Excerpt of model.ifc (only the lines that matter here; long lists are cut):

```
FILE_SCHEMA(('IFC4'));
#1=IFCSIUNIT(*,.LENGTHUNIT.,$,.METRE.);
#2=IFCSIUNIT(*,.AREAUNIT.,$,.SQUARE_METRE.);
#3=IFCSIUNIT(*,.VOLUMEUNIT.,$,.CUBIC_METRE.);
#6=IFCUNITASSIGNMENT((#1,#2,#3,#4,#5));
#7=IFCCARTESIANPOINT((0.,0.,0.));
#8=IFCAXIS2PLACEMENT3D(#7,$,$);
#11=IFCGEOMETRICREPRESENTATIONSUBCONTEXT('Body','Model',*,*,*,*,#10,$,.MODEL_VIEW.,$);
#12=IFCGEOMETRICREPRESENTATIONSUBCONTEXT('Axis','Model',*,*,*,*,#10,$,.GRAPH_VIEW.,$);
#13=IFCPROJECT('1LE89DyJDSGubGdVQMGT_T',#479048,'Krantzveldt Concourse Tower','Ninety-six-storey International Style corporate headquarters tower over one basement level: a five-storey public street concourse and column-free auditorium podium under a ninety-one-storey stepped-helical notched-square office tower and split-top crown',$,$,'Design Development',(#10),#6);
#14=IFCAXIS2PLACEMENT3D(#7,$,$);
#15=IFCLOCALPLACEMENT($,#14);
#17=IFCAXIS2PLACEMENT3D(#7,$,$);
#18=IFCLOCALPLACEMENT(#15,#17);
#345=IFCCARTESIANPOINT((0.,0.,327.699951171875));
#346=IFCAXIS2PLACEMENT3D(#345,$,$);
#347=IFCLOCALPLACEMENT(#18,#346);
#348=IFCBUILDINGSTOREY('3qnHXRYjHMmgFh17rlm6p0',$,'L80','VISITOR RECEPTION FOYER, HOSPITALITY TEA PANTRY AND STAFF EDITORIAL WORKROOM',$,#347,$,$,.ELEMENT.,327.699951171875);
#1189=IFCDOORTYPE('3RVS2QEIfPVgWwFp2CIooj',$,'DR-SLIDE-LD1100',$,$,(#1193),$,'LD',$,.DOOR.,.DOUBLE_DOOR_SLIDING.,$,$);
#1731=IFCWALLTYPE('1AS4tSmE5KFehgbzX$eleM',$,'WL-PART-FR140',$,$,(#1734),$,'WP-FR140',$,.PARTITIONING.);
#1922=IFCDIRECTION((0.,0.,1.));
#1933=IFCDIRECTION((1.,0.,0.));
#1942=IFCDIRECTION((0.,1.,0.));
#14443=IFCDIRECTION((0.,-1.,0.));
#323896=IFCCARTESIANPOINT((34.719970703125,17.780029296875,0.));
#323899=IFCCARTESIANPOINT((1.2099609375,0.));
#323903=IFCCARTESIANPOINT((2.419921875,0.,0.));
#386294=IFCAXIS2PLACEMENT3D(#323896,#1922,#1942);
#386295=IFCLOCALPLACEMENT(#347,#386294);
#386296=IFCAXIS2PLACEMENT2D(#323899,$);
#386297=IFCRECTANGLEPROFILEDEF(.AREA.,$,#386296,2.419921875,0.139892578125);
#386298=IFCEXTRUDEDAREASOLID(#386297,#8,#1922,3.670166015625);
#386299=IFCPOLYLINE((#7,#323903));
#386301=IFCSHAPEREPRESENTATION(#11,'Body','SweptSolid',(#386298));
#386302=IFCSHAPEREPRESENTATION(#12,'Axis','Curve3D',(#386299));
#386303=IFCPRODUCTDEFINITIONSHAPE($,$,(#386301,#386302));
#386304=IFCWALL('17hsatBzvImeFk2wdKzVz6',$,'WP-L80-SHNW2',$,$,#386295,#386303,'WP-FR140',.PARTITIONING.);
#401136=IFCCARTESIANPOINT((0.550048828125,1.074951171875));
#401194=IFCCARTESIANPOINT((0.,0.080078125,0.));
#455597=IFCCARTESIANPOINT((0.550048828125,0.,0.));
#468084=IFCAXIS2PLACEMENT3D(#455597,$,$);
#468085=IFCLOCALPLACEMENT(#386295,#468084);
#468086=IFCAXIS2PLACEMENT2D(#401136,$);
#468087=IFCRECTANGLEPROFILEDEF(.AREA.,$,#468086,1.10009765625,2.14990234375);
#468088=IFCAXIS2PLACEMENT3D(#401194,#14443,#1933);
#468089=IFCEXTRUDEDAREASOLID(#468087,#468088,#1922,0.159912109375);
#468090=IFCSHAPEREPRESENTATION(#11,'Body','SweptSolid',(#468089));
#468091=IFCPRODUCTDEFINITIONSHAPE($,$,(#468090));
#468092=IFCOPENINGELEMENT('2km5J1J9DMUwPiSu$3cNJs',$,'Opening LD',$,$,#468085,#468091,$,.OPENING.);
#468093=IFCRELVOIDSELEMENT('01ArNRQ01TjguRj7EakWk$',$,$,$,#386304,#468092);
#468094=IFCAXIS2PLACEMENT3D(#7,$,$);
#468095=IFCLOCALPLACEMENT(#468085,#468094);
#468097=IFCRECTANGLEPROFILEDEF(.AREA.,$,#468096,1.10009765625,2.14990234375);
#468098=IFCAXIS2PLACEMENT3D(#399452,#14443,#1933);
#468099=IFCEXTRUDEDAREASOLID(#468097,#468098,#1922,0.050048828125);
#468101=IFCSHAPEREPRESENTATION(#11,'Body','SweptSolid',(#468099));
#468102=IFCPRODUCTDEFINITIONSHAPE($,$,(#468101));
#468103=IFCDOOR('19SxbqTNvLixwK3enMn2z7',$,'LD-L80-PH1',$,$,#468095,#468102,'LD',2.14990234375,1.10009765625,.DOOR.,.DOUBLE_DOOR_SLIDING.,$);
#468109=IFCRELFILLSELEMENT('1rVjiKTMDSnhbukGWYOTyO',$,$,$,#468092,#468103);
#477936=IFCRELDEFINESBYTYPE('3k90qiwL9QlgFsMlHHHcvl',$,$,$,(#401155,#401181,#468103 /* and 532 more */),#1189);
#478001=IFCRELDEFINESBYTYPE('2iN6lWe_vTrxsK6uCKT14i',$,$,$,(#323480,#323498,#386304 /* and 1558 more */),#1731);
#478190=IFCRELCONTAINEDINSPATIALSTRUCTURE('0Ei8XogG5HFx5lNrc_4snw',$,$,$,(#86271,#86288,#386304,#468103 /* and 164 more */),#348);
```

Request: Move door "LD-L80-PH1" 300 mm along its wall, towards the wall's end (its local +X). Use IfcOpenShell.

```python
import ifcopenshell
import ifcopenshell.api.geometry
import ifcopenshell.util.placement
import ifcopenshell.util.unit

model = ifcopenshell.open("model.ifc")
unit_scale = ifcopenshell.util.unit.calculate_unit_scale(model)

door = model.by_guid("19SxbqTNvLixwK3enMn2z7")
opening = door.FillsVoids[0].RelatingOpeningElement
wall = opening.VoidsElements[0].RelatingBuildingElement

wall_matrix = ifcopenshell.util.placement.get_local_placement(wall.ObjectPlacement)
shift = wall_matrix[:3, 0] * 0.3 / unit_scale
before = ifcopenshell.util.placement.get_local_placement(door.ObjectPlacement)[:3, 3].copy()

# The door is placed relative to its opening, so it follows when the opening moves.
matrix = ifcopenshell.util.placement.get_local_placement(opening.ObjectPlacement)
matrix[:3, 3] += shift
ifcopenshell.api.geometry.edit_object_placement(
    model, product=opening, matrix=matrix, is_si=False, should_transform_children=True
)

after = ifcopenshell.util.placement.get_local_placement(door.ObjectPlacement)[:3, 3]
print("door moved by", (after - before).round(3) + 0.0)

model.write("model-out.ifc")
```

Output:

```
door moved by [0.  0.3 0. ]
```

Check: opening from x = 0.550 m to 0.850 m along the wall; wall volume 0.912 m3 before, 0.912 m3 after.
